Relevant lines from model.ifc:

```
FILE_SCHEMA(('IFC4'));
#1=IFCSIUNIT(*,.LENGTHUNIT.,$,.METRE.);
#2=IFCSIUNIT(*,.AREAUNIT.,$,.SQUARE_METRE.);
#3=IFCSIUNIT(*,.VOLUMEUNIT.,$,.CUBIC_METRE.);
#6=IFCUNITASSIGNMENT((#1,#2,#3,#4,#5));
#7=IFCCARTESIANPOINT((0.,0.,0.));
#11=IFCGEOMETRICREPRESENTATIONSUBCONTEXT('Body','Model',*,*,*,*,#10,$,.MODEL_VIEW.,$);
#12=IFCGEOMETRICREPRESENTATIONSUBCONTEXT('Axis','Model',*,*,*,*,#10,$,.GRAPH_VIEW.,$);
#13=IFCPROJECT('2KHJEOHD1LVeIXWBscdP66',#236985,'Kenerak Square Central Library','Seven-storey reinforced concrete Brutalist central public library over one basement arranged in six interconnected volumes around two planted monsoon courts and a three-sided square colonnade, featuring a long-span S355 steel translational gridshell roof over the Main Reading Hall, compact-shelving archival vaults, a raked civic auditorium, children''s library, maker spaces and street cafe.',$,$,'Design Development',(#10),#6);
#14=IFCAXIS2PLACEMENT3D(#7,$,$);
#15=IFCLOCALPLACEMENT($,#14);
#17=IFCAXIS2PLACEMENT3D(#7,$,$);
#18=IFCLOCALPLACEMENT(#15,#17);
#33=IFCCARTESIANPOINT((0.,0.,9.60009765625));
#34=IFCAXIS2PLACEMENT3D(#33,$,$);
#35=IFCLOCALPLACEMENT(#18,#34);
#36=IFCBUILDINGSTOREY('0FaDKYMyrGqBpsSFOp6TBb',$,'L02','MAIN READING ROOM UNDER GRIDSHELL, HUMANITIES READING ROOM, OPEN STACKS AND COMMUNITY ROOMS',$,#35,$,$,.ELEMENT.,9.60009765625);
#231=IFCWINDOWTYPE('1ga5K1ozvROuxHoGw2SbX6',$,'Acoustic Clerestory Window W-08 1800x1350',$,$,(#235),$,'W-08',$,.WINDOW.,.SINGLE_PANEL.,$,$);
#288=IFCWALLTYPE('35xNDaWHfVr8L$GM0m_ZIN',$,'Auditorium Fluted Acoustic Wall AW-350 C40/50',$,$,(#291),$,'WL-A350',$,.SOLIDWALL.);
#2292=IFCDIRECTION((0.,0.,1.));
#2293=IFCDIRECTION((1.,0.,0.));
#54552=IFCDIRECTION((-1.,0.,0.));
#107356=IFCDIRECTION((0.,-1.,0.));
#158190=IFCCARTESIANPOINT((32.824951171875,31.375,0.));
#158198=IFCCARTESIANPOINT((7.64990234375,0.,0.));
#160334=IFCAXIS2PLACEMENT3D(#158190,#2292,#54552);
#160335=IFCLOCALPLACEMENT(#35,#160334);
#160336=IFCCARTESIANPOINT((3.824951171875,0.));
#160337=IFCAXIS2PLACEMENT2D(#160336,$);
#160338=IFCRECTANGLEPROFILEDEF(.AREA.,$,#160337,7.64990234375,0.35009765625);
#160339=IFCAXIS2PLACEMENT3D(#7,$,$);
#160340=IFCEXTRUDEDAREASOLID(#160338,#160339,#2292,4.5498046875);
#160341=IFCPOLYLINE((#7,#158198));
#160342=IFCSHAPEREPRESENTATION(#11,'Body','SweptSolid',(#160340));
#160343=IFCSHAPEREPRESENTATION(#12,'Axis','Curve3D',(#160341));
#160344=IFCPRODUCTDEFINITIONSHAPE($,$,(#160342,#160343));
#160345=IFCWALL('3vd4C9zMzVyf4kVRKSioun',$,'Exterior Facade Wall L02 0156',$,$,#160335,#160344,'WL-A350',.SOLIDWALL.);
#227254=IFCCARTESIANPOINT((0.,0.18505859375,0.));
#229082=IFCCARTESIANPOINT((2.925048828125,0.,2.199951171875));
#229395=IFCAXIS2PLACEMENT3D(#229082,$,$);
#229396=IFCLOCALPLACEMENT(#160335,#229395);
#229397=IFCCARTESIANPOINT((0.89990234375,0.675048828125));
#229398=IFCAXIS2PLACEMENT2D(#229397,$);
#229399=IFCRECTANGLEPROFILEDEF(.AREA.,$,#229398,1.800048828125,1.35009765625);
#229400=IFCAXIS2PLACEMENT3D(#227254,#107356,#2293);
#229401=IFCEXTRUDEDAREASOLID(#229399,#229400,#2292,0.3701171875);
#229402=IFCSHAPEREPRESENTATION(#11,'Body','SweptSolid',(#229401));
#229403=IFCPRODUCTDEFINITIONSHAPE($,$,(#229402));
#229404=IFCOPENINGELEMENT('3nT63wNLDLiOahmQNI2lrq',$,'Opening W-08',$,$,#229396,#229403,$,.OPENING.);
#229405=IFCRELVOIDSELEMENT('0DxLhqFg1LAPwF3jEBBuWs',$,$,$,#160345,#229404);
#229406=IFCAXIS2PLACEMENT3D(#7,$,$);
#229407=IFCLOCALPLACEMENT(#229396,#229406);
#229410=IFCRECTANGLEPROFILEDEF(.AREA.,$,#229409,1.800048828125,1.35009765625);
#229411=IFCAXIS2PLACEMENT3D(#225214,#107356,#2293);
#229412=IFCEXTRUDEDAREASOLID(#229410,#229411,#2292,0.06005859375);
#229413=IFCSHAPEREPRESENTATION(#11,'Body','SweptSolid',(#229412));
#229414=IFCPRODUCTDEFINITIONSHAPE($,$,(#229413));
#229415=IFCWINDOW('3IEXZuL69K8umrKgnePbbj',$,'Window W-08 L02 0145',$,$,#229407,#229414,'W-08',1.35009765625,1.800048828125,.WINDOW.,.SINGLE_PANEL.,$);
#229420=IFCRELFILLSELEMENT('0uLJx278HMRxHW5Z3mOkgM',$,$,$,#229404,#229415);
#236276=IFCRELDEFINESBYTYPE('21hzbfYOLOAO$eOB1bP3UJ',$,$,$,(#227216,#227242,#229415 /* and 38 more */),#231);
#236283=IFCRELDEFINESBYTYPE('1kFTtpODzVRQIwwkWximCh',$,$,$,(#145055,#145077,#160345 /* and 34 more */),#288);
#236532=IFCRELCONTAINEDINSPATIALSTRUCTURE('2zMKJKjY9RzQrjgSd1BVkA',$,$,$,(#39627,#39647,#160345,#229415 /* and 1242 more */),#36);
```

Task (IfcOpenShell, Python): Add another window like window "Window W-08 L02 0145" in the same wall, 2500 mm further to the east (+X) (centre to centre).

```python
import ifcopenshell
import ifcopenshell.api.feature
import ifcopenshell.api.geometry
import ifcopenshell.api.root
import ifcopenshell.geom
import ifcopenshell.util.element
import ifcopenshell.util.placement
import ifcopenshell.util.shape

model = ifcopenshell.open("model.ifc")
settings = ifcopenshell.geom.settings()


def volume(element):
    """Net volume in cubic metres, openings subtracted."""
    shape = ifcopenshell.geom.create_shape(settings, element)
    return ifcopenshell.util.shape.get_volume(shape.geometry)


window = model.by_guid("3IEXZuL69K8umrKgnePbbj")
opening = window.FillsVoids[0].RelatingOpeningElement
wall = opening.VoidsElements[0].RelatingBuildingElement
before = volume(wall)
shift = ifcopenshell.util.placement.get_local_placement(wall.ObjectPlacement)[:3, 0] * -2.5

# copy_class copies the void relationship, type, container and properties, but no geometry.
new_opening = ifcopenshell.api.root.copy_class(model, product=opening)
new_opening.Representation = ifcopenshell.util.element.copy_deep(
    model, opening.Representation, exclude=["IfcGeometricRepresentationContext", "IfcRepresentationMap"]
)
new_window = ifcopenshell.api.root.copy_class(model, product=window)
new_window.Representation = ifcopenshell.util.element.copy_deep(
    model, window.Representation, exclude=["IfcGeometricRepresentationContext", "IfcRepresentationMap"]
)
new_window.Tag = None
ifcopenshell.api.feature.add_filling(model, opening=new_opening, element=new_window)

for old, new in ((opening, new_opening), (window, new_window)):
    matrix = ifcopenshell.util.placement.get_local_placement(old.ObjectPlacement)
    matrix[:3, 3] += shift
    ifcopenshell.api.geometry.edit_object_placement(model, product=new, matrix=matrix, is_si=False)

after = volume(wall)

print(f"wall volume {before:.3f} -> {after:.3f} m3")

model.write("model-out.ifc")
```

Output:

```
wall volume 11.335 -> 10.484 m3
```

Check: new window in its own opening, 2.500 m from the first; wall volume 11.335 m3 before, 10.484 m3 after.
